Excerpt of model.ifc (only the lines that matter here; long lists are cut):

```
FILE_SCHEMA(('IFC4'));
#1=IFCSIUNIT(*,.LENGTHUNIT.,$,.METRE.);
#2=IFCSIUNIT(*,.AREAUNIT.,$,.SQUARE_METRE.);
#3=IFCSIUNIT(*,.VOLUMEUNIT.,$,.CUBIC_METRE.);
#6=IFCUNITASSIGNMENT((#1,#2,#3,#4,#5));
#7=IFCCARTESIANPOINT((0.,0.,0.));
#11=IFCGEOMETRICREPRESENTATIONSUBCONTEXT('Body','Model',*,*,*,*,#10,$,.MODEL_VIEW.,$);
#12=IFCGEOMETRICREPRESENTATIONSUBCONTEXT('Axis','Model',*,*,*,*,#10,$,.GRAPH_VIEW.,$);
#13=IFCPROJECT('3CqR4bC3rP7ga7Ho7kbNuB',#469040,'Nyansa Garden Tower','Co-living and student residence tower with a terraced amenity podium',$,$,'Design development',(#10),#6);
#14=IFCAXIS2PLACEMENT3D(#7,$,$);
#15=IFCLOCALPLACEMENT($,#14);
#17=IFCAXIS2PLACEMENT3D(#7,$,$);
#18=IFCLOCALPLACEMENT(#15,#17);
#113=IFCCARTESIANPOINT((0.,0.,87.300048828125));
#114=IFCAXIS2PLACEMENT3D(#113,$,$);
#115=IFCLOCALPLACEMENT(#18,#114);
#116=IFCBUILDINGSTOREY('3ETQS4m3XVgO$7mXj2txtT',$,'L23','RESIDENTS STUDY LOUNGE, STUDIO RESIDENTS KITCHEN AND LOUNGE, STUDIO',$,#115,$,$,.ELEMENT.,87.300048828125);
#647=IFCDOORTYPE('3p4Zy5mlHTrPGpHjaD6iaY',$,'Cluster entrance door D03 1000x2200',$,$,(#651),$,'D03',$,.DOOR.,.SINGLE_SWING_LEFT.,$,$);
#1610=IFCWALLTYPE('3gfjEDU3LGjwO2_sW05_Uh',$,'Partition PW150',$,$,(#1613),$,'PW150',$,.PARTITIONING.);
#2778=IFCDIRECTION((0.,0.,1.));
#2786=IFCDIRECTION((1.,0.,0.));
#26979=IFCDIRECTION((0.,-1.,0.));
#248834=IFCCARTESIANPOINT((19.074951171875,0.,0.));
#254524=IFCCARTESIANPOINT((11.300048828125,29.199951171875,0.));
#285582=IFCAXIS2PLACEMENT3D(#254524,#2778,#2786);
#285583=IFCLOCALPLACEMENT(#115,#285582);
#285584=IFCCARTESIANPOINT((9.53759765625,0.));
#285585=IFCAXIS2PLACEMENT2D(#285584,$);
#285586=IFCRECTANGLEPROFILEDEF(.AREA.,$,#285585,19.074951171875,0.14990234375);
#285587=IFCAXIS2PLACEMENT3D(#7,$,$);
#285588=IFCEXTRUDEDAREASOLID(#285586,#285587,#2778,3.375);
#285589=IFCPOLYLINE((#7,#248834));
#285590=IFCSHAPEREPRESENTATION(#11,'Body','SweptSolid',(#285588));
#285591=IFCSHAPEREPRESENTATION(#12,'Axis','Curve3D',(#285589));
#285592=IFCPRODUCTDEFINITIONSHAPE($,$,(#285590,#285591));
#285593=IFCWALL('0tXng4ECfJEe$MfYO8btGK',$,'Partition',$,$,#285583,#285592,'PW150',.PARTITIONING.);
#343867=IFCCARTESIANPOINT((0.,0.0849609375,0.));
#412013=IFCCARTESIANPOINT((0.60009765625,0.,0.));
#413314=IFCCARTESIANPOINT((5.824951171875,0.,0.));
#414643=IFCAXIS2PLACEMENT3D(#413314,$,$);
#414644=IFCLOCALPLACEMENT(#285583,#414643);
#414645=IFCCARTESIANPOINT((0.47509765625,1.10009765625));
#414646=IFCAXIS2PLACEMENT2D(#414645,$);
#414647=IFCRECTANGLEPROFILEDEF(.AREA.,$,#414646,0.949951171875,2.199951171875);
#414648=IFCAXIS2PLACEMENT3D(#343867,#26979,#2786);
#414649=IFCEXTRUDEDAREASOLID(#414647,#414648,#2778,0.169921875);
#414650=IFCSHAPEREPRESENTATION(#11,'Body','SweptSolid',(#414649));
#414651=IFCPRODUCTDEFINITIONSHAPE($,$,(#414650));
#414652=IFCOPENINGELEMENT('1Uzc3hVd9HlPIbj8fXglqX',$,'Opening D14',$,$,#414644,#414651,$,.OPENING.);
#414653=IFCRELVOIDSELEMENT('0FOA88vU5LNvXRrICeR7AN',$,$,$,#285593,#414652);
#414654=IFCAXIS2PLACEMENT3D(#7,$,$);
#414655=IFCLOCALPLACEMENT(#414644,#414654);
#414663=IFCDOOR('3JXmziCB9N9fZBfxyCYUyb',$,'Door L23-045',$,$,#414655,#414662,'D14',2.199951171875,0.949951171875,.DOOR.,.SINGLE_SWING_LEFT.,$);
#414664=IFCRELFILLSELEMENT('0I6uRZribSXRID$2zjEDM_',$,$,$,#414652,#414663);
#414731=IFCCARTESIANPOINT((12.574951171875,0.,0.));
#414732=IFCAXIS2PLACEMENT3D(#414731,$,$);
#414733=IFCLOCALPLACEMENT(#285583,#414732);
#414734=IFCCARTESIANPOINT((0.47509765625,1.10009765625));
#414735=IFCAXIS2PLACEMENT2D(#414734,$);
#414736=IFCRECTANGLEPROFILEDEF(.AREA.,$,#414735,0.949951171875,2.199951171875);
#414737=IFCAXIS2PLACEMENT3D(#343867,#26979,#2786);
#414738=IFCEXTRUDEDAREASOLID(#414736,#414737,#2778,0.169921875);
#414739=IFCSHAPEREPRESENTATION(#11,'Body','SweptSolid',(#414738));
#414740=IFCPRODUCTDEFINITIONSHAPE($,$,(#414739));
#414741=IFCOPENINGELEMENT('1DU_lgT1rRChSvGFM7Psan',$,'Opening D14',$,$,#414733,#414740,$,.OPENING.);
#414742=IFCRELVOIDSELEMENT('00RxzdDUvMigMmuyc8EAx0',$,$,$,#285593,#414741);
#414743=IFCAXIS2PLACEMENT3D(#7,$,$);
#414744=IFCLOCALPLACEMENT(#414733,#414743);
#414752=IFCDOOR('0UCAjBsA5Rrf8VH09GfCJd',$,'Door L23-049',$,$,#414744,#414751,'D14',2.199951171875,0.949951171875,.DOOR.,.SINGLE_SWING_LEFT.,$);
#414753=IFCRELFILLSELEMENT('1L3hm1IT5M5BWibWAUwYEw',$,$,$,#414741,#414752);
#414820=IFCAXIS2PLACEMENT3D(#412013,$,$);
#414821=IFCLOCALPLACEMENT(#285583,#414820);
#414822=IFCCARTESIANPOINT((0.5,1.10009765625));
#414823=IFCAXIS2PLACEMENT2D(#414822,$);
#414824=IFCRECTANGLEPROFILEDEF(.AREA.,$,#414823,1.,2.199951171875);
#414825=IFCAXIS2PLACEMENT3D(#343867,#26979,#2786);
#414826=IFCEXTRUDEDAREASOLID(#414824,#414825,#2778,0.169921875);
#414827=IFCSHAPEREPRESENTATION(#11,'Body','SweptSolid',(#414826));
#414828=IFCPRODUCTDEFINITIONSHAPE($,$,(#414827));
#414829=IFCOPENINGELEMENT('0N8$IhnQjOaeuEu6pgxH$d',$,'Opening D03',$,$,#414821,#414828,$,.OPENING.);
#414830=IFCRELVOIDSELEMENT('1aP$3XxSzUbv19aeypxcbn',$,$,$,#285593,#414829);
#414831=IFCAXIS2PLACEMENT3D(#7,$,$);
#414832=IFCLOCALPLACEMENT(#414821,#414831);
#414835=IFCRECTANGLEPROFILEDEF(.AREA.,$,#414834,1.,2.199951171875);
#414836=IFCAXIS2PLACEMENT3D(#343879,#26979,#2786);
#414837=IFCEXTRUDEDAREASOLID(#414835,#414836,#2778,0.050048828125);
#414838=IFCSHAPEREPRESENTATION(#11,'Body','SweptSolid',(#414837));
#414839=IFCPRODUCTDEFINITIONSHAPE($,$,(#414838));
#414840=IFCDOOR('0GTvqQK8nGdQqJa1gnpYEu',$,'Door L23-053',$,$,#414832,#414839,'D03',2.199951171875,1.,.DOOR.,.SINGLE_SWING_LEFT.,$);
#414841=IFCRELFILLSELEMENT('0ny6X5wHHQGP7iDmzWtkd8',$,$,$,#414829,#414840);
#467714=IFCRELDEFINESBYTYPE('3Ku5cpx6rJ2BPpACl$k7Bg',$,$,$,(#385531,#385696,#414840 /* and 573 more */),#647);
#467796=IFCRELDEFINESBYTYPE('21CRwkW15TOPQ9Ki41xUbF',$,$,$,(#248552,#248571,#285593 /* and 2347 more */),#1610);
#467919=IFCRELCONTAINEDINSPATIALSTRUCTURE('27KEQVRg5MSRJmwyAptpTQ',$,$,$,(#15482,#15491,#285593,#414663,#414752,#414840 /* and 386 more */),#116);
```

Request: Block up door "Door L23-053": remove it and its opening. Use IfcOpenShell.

```python
import ifcopenshell
import ifcopenshell.api.feature
import ifcopenshell.api.root
import ifcopenshell.geom
import ifcopenshell.util.shape

model = ifcopenshell.open("model.ifc")
settings = ifcopenshell.geom.settings()


def volume(element):
    """Net volume in cubic metres, openings subtracted."""
    shape = ifcopenshell.geom.create_shape(settings, element)
    return ifcopenshell.util.shape.get_volume(shape.geometry)


door = model.by_guid("0GTvqQK8nGdQqJa1gnpYEu")
opening = door.FillsVoids[0].RelatingOpeningElement
wall = opening.VoidsElements[0].RelatingBuildingElement
before = volume(wall)

ifcopenshell.api.root.remove_product(model, product=door)
ifcopenshell.api.feature.remove_feature(model, feature=opening)

after = volume(wall)

print(f"wall volume {before:.3f} -> {after:.3f} m3")

model.write("model_edited.ifc")
```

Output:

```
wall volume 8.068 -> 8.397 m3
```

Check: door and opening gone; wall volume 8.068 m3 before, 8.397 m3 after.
